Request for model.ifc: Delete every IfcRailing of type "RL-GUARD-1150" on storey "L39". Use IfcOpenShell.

First a look at what the model holds.

```python
import ifcopenshell
import ifcopenshell.util.element

model = ifcopenshell.open("model.ifc")
print(model.schema)
storey = next(s for s in model.by_type("IfcBuildingStorey") if s.Name == "L39")
railings = [e for e in ifcopenshell.util.element.get_decomposition(storey) if e.is_a("IfcRailing")]
seen = {}
for e in railings:
    element_type = ifcopenshell.util.element.get_type(e)
    name = element_type.Name if element_type not in (None, e) else None
    seen[name] = seen.get(name, 0) + 1
for name, count in sorted(seen.items(), key=str):
    print(count, "x", name)
```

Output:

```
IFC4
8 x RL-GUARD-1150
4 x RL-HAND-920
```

```python
import ifcopenshell
import ifcopenshell.api.root
import ifcopenshell.util.element

model = ifcopenshell.open("model.ifc")

storey = next(s for s in model.by_type("IfcBuildingStorey") if s.Name == "L39")
railings = [e for e in ifcopenshell.util.element.get_decomposition(storey) if e.is_a("IfcRailing")]
targets = [e for e in railings if (t := ifcopenshell.util.element.get_type(e)) not in (None, e) and t.Name == "RL-GUARD-1150"]

for e in targets:
    ifcopenshell.api.root.remove_product(model, product=e)
print(len(targets), "removed")

model.write("model_rev.ifc")
```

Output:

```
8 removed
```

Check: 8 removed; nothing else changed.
